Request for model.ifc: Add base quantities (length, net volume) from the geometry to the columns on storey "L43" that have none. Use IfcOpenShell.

First a look at what the model holds.

```python
import ifcopenshell
import ifcopenshell.util.element
import ifcopenshell.util.unit

model = ifcopenshell.open("model.ifc")
print(model.schema)
for unit_type in ("LENGTHUNIT", "AREAUNIT", "VOLUMEUNIT"):
    print(unit_type, ifcopenshell.util.unit.calculate_unit_scale(model, unit_type))
storey = next(s for s in model.by_type("IfcBuildingStorey") if s.Name == "L43")
columns = [e for e in ifcopenshell.util.element.get_decomposition(storey) if e.is_a("IfcColumn")]
for e in sorted(columns, key=lambda e: e.id()):
    print(e.id(), e.is_a(), e.Name, list(ifcopenshell.util.element.get_psets(e, qtos_only=True)), sep=" | ")
```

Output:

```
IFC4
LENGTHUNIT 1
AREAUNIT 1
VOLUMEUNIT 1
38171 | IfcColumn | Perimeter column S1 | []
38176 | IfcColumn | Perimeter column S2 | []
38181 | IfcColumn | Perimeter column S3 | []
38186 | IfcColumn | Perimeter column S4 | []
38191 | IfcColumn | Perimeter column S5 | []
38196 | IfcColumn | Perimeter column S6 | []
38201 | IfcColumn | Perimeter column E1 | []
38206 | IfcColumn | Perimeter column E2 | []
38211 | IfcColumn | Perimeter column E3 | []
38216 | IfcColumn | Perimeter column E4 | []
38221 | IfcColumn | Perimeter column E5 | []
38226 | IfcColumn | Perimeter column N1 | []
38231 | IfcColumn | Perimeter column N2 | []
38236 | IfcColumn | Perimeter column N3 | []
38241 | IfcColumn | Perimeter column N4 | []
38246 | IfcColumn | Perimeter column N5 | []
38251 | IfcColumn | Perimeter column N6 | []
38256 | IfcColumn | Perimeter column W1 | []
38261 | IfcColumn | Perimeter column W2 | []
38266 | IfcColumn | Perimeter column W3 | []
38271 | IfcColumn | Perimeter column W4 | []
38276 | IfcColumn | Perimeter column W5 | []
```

```python
import ifcopenshell
import ifcopenshell.api.pset
import ifcopenshell.geom
import ifcopenshell.util.element
import ifcopenshell.util.shape
import ifcopenshell.util.unit

model = ifcopenshell.open("model.ifc")
unit_scale = ifcopenshell.util.unit.calculate_unit_scale(model)
volume_scale = ifcopenshell.util.unit.calculate_unit_scale(model, "VOLUMEUNIT")
settings = ifcopenshell.geom.settings()

storey = next(s for s in model.by_type("IfcBuildingStorey") if s.Name == "L43")
columns = [e for e in ifcopenshell.util.element.get_decomposition(storey) if e.is_a("IfcColumn")]

for e in sorted(columns, key=lambda e: e.id()):
    if ifcopenshell.util.element.get_psets(e, qtos_only=True, should_inherit=False):
        continue
    # Geometry comes back in metres, in the element's own axes.
    shape = ifcopenshell.geom.create_shape(settings, e)
    values = {
        "Length": ifcopenshell.util.shape.get_z(shape.geometry) / unit_scale,
        "NetVolume": ifcopenshell.util.shape.get_volume(shape.geometry) / volume_scale,
    }
    qto = ifcopenshell.api.pset.add_qto(model, product=e, name="Qto_ColumnBaseQuantities")
    ifcopenshell.api.pset.edit_qto(model, qto=qto, properties=values)
    print(e.id(), {k: round(v, 3) for k, v in values.items()})

model.write("model_v2.ifc")
```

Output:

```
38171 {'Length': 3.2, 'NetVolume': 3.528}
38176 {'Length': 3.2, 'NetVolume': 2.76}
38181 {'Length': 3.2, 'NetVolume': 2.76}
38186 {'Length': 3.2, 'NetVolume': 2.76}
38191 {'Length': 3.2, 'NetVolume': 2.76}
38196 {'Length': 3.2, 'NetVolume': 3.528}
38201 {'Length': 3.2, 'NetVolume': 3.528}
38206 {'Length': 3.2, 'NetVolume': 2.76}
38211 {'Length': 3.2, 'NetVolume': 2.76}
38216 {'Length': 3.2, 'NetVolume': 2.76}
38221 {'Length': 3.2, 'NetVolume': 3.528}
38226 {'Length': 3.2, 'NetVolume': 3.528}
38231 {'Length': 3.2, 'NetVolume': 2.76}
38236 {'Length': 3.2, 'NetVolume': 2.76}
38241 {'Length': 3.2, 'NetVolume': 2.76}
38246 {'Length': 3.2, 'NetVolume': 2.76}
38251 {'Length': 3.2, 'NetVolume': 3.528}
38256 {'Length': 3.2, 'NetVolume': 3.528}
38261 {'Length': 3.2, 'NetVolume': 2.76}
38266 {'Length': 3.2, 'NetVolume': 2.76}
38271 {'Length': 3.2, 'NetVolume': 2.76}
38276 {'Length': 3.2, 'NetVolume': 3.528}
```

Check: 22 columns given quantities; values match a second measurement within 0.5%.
